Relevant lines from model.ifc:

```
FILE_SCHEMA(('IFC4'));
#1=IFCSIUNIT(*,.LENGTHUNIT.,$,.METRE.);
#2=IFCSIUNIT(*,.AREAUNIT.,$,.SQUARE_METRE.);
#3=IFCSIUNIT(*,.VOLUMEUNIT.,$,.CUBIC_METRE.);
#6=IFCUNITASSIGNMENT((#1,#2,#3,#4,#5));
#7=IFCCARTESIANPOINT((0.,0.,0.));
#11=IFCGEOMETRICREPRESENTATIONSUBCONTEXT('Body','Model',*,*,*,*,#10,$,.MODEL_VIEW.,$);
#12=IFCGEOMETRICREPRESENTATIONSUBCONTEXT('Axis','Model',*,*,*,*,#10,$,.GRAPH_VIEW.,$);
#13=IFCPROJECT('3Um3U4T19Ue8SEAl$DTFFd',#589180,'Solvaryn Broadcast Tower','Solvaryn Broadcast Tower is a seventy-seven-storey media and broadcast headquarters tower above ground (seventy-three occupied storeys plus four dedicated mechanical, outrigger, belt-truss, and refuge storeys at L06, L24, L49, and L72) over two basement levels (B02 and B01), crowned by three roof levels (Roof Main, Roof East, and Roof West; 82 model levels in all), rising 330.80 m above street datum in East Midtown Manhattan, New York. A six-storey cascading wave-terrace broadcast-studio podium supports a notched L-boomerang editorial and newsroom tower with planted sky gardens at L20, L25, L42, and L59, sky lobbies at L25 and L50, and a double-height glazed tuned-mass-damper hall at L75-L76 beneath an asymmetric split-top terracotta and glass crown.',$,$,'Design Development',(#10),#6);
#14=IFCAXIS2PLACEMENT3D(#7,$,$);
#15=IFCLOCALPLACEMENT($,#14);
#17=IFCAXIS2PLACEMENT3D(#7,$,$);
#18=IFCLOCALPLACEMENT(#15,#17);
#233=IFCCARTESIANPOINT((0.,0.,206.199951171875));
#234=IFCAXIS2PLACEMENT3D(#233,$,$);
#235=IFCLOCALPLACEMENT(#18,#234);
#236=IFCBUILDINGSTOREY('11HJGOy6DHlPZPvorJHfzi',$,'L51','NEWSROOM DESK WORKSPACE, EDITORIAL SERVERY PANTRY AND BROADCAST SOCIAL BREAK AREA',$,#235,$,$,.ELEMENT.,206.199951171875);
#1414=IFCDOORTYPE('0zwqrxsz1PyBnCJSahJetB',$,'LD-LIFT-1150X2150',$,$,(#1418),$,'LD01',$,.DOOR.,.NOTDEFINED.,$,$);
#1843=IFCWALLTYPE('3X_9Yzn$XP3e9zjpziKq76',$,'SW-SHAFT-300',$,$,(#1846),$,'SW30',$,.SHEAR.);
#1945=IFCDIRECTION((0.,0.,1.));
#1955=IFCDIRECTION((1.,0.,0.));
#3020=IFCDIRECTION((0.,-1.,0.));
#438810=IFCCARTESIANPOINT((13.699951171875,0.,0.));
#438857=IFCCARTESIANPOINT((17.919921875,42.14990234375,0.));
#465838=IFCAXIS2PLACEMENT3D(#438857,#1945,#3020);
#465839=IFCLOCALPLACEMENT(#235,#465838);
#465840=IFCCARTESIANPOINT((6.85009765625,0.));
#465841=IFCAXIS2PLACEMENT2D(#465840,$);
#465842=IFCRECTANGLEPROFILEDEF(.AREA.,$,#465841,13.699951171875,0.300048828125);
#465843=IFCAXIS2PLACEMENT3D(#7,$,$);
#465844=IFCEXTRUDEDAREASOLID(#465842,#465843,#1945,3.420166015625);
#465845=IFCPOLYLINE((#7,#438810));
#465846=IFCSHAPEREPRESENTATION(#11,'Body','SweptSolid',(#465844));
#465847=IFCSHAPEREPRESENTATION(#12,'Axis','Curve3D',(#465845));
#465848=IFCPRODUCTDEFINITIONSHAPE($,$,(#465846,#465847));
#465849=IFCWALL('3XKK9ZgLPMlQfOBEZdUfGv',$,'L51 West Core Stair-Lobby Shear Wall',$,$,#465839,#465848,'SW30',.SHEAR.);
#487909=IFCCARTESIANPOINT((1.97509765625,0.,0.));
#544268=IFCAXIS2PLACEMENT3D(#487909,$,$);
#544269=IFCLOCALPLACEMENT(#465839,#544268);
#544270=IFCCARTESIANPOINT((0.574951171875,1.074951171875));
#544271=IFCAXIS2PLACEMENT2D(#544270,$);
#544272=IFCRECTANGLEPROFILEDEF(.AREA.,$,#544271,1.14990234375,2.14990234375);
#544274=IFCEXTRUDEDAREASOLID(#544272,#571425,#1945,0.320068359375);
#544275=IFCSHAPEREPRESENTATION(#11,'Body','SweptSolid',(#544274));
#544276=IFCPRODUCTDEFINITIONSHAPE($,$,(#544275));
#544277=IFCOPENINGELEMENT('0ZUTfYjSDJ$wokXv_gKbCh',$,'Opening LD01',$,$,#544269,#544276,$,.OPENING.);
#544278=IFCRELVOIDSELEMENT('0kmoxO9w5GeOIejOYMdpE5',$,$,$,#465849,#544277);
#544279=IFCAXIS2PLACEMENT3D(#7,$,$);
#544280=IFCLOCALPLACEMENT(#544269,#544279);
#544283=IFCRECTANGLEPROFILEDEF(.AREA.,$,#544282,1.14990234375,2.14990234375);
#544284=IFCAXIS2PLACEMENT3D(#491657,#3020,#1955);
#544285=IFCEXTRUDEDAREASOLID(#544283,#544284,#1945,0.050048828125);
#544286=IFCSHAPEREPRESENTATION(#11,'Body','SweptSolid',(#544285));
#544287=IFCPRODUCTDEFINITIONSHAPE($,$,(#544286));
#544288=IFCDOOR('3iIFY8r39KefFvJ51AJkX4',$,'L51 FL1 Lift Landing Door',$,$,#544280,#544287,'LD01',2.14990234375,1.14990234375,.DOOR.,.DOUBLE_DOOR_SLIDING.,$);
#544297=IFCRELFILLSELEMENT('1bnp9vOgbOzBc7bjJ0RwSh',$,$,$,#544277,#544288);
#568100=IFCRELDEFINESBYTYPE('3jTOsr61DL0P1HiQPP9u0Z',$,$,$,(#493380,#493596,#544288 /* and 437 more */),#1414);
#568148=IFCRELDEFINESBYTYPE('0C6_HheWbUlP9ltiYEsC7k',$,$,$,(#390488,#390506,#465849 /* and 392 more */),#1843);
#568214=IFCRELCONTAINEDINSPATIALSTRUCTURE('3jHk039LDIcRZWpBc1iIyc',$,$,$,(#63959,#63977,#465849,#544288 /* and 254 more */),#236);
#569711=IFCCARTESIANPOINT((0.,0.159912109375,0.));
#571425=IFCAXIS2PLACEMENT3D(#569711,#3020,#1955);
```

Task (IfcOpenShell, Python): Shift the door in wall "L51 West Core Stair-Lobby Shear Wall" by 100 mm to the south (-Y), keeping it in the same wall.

```python
import ifcopenshell
import ifcopenshell.api.geometry
import ifcopenshell.util.placement
import ifcopenshell.util.unit

model = ifcopenshell.open("model.ifc")
unit_scale = ifcopenshell.util.unit.calculate_unit_scale(model)

door = model.by_id(544288)
opening = door.FillsVoids[0].RelatingOpeningElement
wall = opening.VoidsElements[0].RelatingBuildingElement

wall_matrix = ifcopenshell.util.placement.get_local_placement(wall.ObjectPlacement)
shift = wall_matrix[:3, 0] * 0.1 / unit_scale
before = ifcopenshell.util.placement.get_local_placement(door.ObjectPlacement)[:3, 3].copy()

# The door is placed relative to its opening, so it follows when the opening moves.
matrix = ifcopenshell.util.placement.get_local_placement(opening.ObjectPlacement)
matrix[:3, 3] += shift
ifcopenshell.api.geometry.edit_object_placement(
    model, product=opening, matrix=matrix, is_si=False, should_transform_children=True
)

after = ifcopenshell.util.placement.get_local_placement(door.ObjectPlacement)[:3, 3]
print("door moved by", (after - before).round(3) + 0.0)

model.write("model_rev.ifc")
```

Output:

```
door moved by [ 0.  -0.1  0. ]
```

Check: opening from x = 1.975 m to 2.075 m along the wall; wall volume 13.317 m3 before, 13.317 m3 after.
